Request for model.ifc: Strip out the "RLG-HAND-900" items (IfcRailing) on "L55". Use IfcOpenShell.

First a look at what the model holds.

```python
import ifcopenshell
import ifcopenshell.util.element

model = ifcopenshell.open("model.ifc")
print(model.schema)
storey = next(s for s in model.by_type("IfcBuildingStorey") if s.Name == "L55")
railings = [e for e in ifcopenshell.util.element.get_decomposition(storey) if e.is_a("IfcRailing")]
seen = {}
for e in railings:
    element_type = ifcopenshell.util.element.get_type(e)
    name = element_type.Name if element_type not in (None, e) else None
    seen[name] = seen.get(name, 0) + 1
for name, count in sorted(seen.items(), key=str):
    print(count, "x", name)
```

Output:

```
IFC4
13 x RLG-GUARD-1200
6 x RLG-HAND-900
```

```python
import ifcopenshell
import ifcopenshell.api.root
import ifcopenshell.util.element

model = ifcopenshell.open("model.ifc")

storey = next(s for s in model.by_type("IfcBuildingStorey") if s.Name == "L55")
railings = [e for e in ifcopenshell.util.element.get_decomposition(storey) if e.is_a("IfcRailing")]
targets = [e for e in railings if (t := ifcopenshell.util.element.get_type(e)) not in (None, e) and t.Name == "RLG-HAND-900"]

for e in targets:
    ifcopenshell.api.root.remove_product(model, product=e)
print(len(targets), "removed")

model.write("model_rev.ifc")
```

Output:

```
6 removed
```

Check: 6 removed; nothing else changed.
